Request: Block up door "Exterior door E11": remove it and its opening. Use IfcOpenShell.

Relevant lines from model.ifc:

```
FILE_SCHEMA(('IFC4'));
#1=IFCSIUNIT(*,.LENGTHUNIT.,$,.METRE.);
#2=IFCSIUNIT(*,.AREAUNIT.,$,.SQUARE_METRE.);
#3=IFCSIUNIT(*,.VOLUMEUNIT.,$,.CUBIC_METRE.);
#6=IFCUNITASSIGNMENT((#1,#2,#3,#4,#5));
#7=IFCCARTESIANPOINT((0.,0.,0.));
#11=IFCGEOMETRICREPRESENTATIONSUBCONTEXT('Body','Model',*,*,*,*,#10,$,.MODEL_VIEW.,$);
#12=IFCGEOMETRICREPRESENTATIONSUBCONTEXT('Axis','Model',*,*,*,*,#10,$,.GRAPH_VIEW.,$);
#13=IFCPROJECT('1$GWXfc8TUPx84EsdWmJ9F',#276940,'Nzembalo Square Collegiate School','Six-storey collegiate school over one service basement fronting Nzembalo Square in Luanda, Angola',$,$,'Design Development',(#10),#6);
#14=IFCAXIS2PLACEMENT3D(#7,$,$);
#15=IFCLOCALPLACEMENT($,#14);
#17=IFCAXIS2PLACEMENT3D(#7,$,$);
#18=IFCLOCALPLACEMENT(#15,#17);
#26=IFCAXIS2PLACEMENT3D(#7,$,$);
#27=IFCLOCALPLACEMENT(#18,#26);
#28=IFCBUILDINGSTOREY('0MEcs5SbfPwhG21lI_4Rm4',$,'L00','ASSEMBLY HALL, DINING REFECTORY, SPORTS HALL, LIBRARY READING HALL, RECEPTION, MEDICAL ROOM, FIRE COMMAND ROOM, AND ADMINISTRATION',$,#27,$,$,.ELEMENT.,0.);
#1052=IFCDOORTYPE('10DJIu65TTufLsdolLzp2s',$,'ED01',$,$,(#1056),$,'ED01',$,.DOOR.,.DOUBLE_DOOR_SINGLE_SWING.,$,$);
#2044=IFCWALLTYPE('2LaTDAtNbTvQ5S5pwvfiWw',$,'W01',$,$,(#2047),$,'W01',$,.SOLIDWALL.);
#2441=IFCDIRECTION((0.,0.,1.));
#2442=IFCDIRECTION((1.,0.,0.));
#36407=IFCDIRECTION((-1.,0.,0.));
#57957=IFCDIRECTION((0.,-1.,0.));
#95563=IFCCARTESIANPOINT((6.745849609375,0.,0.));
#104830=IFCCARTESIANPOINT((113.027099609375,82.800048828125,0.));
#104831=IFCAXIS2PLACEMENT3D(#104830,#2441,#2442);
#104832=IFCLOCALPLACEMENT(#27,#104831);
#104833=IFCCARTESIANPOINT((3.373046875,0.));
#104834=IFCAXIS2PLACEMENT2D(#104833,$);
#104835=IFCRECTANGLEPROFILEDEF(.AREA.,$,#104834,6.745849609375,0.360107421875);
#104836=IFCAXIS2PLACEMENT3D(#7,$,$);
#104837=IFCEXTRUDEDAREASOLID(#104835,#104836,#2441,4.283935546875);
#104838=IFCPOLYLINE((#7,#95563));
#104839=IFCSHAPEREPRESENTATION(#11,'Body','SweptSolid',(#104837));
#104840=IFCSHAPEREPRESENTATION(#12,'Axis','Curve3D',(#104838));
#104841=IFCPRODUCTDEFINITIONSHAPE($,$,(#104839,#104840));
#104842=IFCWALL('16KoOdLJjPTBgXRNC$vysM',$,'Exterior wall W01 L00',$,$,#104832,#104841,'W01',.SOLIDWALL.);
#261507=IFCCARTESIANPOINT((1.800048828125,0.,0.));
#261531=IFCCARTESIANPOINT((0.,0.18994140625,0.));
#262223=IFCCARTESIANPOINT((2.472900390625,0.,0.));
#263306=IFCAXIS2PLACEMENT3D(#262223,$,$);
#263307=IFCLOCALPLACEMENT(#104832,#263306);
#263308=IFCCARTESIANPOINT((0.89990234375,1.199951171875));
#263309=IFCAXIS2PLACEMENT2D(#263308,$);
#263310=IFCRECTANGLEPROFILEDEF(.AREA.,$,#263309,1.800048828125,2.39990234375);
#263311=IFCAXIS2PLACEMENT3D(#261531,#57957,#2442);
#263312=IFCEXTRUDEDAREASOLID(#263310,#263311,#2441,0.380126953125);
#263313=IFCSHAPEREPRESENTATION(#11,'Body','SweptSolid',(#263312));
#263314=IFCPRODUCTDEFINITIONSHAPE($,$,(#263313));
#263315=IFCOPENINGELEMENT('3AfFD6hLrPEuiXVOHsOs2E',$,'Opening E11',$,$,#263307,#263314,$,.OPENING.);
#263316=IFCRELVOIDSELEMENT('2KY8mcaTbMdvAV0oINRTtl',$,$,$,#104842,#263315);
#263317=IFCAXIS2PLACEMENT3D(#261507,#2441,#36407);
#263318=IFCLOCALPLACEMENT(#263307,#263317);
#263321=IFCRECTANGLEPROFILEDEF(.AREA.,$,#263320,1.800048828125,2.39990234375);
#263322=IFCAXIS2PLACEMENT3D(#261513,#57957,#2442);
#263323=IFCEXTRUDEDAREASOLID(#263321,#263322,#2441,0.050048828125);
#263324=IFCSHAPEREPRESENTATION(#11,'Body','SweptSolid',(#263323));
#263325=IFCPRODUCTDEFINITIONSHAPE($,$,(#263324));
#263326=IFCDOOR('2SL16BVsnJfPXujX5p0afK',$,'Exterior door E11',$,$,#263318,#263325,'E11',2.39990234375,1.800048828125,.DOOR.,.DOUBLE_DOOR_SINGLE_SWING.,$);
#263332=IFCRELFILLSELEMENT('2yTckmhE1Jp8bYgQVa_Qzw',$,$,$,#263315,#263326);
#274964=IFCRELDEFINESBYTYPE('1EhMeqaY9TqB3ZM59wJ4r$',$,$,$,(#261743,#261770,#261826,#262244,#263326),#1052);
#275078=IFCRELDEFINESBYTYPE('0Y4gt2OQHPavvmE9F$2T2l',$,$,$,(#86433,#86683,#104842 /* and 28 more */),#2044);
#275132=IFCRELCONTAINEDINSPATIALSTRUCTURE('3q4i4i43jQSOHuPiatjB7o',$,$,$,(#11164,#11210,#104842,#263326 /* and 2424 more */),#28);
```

```python
import ifcopenshell
import ifcopenshell.api.feature
import ifcopenshell.api.root
import ifcopenshell.geom
import ifcopenshell.util.shape

model = ifcopenshell.open("model.ifc")
settings = ifcopenshell.geom.settings()


def volume(element):
    """Net volume in cubic metres, openings subtracted."""
    shape = ifcopenshell.geom.create_shape(settings, element)
    return ifcopenshell.util.shape.get_volume(shape.geometry)


door = model.by_guid("2SL16BVsnJfPXujX5p0afK")
opening = door.FillsVoids[0].RelatingOpeningElement
wall = opening.VoidsElements[0].RelatingBuildingElement
before = volume(wall)

ifcopenshell.api.root.remove_product(model, product=door)
ifcopenshell.api.feature.remove_feature(model, feature=opening)

after = volume(wall)

print(f"wall volume {before:.3f} -> {after:.3f} m3")

model.write("model_v2.ifc")
```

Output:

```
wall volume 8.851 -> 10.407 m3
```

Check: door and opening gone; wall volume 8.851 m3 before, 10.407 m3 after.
